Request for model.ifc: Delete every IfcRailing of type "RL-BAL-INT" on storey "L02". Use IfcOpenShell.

First a look at what the model holds.

```python
import ifcopenshell
import ifcopenshell.util.element

model = ifcopenshell.open("model.ifc")
print(model.schema)
storey = next(s for s in model.by_type("IfcBuildingStorey") if s.Name == "L02")
railings = [e for e in ifcopenshell.util.element.get_decomposition(storey) if e.is_a("IfcRailing")]
seen = {}
for e in railings:
    element_type = ifcopenshell.util.element.get_type(e)
    name = element_type.Name if element_type not in (None, e) else None
    seen[name] = seen.get(name, 0) + 1
for name, count in sorted(seen.items(), key=str):
    print(count, "x", name)
```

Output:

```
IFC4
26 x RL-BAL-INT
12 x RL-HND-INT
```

```python
import ifcopenshell
import ifcopenshell.api.root
import ifcopenshell.util.element

model = ifcopenshell.open("model.ifc")

storey = next(s for s in model.by_type("IfcBuildingStorey") if s.Name == "L02")
railings = [e for e in ifcopenshell.util.element.get_decomposition(storey) if e.is_a("IfcRailing")]
targets = [e for e in railings if (t := ifcopenshell.util.element.get_type(e)) not in (None, e) and t.Name == "RL-BAL-INT"]

for e in targets:
    ifcopenshell.api.root.remove_product(model, product=e)
print(len(targets), "removed")

model.write("model_v2.ifc")
```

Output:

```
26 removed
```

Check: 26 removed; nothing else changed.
